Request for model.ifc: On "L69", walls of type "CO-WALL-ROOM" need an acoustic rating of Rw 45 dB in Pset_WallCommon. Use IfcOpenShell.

First a look at what the model holds.

```python
import ifcopenshell
import ifcopenshell.util.element

model = ifcopenshell.open("model.ifc")
print(model.schema)
storey = next(s for s in model.by_type("IfcBuildingStorey") if s.Name == "L69")
walls = [e for e in ifcopenshell.util.element.get_decomposition(storey) if e.is_a("IfcWall")]
seen = {}
for e in walls:
    element_type = ifcopenshell.util.element.get_type(e)
    key = (element_type.Name if element_type != e and element_type else None, ifcopenshell.util.element.get_pset(e, "Pset_WallCommon", "AcousticRating"))
    seen[key] = seen.get(key, 0) + 1
for (name, value), count in sorted(seen.items(), key=str):
    print(count, "x", name, "|", value)
```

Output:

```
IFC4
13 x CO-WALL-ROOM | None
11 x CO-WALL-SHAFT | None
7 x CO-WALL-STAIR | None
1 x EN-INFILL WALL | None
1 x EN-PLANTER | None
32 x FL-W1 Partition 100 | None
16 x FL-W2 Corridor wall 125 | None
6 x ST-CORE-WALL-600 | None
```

```python
import ifcopenshell
import ifcopenshell.api.pset
import ifcopenshell.util.element

model = ifcopenshell.open("model.ifc")

storey = next(s for s in model.by_type("IfcBuildingStorey") if s.Name == "L69")
walls = [e for e in ifcopenshell.util.element.get_decomposition(storey) if e.is_a("IfcWall")]

count = 0
for e in walls:
    element_type = ifcopenshell.util.element.get_type(e)
    if element_type in (None, e) or element_type.Name != "CO-WALL-ROOM":
        continue
    found = ifcopenshell.util.element.get_pset(e, "Pset_WallCommon", should_inherit=False)
    if found:
        pset = model.by_id(found["id"])
        if len(ifcopenshell.util.element.get_elements_by_pset(pset)) > 1:
            pset = ifcopenshell.api.pset.unshare_pset(model, products=[e], pset=pset)[0]
    else:
        pset = ifcopenshell.api.pset.add_pset(model, product=e, name="Pset_WallCommon")
    ifcopenshell.api.pset.edit_pset(model, pset=pset, properties={"AcousticRating": "Rw 45 dB"})
    count += 1

print(count, "walls updated")

model.write("model_updated.ifc")
```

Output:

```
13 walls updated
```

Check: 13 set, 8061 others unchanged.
